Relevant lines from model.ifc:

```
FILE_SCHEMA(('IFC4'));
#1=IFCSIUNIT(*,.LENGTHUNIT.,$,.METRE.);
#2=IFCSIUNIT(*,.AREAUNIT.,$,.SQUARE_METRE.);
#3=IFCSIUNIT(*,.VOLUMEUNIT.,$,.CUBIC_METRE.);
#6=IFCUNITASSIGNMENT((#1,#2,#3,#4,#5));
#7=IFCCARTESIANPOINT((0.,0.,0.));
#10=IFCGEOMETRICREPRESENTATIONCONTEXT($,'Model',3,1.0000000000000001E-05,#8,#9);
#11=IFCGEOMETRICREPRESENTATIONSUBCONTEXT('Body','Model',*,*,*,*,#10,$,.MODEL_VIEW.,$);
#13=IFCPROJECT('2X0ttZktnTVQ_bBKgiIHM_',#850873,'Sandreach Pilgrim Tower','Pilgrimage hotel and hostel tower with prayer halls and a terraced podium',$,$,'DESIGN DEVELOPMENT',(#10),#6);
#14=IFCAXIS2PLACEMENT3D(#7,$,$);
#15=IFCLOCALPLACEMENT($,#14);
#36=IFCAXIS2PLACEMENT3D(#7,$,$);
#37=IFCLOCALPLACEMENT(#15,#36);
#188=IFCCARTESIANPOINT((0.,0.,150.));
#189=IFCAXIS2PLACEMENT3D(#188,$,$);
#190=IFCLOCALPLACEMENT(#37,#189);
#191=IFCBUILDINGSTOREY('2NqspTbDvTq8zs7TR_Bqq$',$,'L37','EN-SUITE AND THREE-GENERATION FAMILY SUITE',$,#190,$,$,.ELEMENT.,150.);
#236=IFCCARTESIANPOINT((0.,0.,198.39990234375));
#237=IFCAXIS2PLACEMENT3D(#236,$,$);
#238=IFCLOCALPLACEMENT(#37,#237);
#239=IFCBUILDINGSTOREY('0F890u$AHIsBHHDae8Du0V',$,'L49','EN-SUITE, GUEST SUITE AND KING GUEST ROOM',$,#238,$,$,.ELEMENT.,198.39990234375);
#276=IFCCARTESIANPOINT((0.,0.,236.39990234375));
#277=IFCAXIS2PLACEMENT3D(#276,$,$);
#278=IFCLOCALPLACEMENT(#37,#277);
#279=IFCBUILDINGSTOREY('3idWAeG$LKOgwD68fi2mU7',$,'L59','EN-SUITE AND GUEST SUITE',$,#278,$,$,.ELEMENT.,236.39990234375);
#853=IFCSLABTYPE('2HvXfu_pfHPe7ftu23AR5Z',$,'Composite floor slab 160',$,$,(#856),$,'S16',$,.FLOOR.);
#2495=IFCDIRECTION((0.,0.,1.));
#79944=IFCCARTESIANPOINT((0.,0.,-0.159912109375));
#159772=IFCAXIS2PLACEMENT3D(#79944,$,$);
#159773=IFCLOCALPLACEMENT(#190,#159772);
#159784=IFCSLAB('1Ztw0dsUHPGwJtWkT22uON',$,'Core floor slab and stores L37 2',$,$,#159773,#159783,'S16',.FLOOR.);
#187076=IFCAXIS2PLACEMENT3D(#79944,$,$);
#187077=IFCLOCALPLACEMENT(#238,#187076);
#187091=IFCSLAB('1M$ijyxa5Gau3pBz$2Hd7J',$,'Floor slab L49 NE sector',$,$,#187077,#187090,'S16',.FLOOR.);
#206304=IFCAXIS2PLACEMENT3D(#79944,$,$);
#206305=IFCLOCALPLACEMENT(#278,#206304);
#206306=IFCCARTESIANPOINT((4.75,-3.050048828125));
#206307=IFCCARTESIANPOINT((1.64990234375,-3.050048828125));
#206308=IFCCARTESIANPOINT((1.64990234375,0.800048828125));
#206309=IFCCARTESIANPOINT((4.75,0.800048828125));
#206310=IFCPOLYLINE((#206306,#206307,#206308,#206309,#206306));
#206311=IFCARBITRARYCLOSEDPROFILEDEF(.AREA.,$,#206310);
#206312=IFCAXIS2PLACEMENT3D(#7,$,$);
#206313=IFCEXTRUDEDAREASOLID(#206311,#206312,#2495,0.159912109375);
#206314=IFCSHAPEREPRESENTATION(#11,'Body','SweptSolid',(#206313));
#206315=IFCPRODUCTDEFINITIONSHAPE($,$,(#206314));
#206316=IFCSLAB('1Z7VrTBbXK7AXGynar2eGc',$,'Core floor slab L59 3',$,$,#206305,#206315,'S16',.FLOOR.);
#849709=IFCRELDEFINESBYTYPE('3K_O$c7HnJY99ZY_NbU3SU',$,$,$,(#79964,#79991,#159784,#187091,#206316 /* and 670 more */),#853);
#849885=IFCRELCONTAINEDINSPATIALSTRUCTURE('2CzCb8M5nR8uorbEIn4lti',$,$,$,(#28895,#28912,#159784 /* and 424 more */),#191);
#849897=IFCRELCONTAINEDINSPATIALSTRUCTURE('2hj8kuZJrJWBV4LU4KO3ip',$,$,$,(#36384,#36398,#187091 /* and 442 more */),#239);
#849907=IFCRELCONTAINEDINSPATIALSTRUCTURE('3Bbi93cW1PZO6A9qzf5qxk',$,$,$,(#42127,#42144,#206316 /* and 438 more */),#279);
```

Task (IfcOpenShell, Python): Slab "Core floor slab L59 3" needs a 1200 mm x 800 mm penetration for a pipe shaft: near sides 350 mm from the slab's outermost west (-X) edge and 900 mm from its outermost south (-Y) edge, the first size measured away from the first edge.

```python
import numpy as np
import ifcopenshell
import ifcopenshell.api.feature
import ifcopenshell.api.geometry
import ifcopenshell.api.root
import ifcopenshell.geom
import ifcopenshell.util.placement
import ifcopenshell.util.representation
import ifcopenshell.util.shape
import ifcopenshell.util.unit

model = ifcopenshell.open("model.ifc")
unit_scale = ifcopenshell.util.unit.calculate_unit_scale(model)
settings = ifcopenshell.geom.settings()


def volume(element):
    """Net volume in cubic metres, openings subtracted."""
    shape = ifcopenshell.geom.create_shape(settings, element)
    return ifcopenshell.util.shape.get_volume(shape.geometry)


slab = model.by_guid("1Z7VrTBbXK7AXGynar2eGc")
before = volume(slab)

# Extent in the slab's own axes, in metres. The edges named are its -X and -Y sides.
slab_shape = ifcopenshell.geom.create_shape(settings, slab)
vertices = ifcopenshell.util.shape.get_vertices(slab_shape.geometry)
x_min, y_min, bottom = vertices.min(axis=0)
top = vertices[:, 2].max()

opening = ifcopenshell.api.root.create_entity(model, ifc_class="IfcOpeningElement", name="Pipe shaft opening", predefined_type="OPENING")
context = ifcopenshell.util.representation.get_context(model, "Model", "Body", "MODEL_VIEW")
width, depth = 1.2, 0.8
outline = [(0.0, 0.0), (width, 0.0), (width, depth), (0.0, depth), (0.0, 0.0)]
# Overshoot both faces by 50 mm so the cut is clean.
shape = ifcopenshell.api.geometry.add_slab_representation(
    model, context=context, depth=top - bottom + 0.1, polyline=outline
)
ifcopenshell.api.geometry.assign_representation(model, product=opening, representation=shape)

matrix = ifcopenshell.util.placement.get_local_placement(slab.ObjectPlacement)
matrix[:, 3] = matrix @ np.append(np.array([x_min + 0.35, y_min + 0.9, bottom - 0.05]) / unit_scale, 1.0)
ifcopenshell.api.geometry.edit_object_placement(model, product=opening, matrix=matrix, is_si=False)
ifcopenshell.api.feature.add_feature(model, feature=opening, element=slab)

after = volume(slab)

print(f"slab volume {before:.3f} -> {after:.3f} m3")

model.write("model_edited.ifc")
```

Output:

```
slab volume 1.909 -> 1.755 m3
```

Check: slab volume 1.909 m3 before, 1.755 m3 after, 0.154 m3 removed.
